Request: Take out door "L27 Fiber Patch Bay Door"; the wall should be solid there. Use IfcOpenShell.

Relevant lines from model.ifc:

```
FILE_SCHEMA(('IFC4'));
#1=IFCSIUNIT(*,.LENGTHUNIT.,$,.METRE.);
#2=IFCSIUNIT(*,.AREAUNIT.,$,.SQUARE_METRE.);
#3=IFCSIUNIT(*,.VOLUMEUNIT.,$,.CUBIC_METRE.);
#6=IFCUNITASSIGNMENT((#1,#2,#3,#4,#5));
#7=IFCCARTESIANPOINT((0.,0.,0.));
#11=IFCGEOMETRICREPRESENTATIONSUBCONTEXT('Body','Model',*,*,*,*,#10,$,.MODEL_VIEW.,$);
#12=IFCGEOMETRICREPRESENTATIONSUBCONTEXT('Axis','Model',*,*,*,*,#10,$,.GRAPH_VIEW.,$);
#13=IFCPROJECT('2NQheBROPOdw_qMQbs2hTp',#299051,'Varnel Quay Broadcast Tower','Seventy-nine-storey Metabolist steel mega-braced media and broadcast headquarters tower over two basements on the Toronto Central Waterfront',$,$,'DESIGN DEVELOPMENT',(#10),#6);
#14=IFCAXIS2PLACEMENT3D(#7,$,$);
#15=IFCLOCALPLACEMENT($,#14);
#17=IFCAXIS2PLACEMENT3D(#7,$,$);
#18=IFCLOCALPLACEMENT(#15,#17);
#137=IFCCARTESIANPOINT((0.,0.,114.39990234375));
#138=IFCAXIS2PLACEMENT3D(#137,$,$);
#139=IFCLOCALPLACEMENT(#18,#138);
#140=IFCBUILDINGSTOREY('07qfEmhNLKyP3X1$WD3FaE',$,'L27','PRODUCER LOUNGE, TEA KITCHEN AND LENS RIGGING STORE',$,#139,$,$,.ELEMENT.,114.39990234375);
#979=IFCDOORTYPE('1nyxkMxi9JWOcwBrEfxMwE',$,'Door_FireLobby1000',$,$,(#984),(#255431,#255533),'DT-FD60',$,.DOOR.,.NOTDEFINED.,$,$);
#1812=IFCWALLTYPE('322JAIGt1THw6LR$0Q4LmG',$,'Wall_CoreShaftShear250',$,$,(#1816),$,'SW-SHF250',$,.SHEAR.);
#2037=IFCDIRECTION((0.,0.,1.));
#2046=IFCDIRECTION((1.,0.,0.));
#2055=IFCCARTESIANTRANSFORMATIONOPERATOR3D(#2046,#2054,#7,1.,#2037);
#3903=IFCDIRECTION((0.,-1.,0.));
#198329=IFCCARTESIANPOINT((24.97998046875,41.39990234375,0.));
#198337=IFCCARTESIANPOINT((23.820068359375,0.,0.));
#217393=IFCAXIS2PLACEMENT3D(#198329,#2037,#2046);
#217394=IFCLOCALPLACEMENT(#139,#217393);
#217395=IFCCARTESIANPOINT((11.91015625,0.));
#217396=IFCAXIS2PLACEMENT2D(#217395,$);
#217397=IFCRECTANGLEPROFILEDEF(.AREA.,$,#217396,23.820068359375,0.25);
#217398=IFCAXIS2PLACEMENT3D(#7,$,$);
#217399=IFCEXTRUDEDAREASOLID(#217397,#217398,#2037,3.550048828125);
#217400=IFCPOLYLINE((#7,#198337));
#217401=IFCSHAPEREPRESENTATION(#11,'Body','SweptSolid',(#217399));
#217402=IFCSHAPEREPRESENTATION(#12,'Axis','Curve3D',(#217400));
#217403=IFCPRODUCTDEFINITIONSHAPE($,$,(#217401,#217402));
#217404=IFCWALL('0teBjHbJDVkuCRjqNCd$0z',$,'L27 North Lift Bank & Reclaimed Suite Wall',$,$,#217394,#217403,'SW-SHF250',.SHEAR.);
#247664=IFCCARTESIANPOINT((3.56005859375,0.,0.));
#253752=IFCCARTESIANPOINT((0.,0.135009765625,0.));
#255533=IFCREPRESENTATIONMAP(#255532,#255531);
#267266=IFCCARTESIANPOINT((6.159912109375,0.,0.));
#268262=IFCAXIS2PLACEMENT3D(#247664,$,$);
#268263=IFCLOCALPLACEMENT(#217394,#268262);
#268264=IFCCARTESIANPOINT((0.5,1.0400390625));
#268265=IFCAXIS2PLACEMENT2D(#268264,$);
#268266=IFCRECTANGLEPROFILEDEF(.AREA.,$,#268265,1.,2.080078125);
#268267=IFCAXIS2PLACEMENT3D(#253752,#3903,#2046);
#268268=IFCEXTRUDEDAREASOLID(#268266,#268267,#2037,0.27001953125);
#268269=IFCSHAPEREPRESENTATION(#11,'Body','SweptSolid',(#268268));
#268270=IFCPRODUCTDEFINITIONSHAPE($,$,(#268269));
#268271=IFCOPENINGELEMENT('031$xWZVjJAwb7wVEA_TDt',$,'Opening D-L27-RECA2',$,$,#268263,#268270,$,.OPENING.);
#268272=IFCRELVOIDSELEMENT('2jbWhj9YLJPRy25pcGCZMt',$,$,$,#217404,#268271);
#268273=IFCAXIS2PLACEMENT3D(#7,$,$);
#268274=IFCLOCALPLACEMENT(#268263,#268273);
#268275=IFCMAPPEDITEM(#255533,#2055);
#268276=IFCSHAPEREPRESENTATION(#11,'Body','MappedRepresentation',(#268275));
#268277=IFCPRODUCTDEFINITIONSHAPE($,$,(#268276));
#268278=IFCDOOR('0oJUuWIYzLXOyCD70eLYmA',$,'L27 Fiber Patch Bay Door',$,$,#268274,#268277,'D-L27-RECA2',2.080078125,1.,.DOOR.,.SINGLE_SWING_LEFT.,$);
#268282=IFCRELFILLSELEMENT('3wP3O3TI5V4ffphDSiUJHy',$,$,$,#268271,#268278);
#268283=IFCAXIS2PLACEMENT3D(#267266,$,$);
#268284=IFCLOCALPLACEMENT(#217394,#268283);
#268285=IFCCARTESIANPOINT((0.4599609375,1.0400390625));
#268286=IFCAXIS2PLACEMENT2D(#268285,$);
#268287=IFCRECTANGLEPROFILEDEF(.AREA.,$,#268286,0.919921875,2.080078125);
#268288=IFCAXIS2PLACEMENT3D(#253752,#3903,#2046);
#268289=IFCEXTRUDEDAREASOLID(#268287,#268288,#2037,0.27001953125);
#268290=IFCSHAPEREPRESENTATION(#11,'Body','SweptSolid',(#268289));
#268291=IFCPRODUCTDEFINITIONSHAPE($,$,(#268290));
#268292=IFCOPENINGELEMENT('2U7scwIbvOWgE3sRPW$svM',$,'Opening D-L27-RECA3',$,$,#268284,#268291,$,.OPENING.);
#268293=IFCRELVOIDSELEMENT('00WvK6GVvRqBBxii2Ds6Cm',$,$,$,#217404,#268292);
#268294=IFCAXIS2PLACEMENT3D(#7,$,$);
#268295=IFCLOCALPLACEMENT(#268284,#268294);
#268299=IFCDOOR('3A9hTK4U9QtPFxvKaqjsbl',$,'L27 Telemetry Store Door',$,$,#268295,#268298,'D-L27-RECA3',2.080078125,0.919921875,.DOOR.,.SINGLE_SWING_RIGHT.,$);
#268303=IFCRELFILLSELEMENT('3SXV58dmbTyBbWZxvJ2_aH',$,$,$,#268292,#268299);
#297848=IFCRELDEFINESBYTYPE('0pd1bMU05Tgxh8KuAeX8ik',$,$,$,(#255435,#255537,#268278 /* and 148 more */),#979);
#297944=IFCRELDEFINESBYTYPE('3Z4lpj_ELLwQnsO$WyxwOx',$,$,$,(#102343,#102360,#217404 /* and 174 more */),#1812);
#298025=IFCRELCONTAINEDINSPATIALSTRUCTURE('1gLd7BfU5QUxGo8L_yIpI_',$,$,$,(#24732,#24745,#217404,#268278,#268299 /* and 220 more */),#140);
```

```python
import ifcopenshell
import ifcopenshell.api.feature
import ifcopenshell.api.root
import ifcopenshell.geom
import ifcopenshell.util.shape

model = ifcopenshell.open("model.ifc")
settings = ifcopenshell.geom.settings()


def volume(element):
    """Net volume in cubic metres, openings subtracted."""
    shape = ifcopenshell.geom.create_shape(settings, element)
    return ifcopenshell.util.shape.get_volume(shape.geometry)


door = model.by_guid("0oJUuWIYzLXOyCD70eLYmA")
opening = door.FillsVoids[0].RelatingOpeningElement
wall = opening.VoidsElements[0].RelatingBuildingElement
before = volume(wall)

ifcopenshell.api.root.remove_product(model, product=door)
ifcopenshell.api.feature.remove_feature(model, feature=opening)

after = volume(wall)

print(f"wall volume {before:.3f} -> {after:.3f} m3")

model.write("model-out.ifc")
```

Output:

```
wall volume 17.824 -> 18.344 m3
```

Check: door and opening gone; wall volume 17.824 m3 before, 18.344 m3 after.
